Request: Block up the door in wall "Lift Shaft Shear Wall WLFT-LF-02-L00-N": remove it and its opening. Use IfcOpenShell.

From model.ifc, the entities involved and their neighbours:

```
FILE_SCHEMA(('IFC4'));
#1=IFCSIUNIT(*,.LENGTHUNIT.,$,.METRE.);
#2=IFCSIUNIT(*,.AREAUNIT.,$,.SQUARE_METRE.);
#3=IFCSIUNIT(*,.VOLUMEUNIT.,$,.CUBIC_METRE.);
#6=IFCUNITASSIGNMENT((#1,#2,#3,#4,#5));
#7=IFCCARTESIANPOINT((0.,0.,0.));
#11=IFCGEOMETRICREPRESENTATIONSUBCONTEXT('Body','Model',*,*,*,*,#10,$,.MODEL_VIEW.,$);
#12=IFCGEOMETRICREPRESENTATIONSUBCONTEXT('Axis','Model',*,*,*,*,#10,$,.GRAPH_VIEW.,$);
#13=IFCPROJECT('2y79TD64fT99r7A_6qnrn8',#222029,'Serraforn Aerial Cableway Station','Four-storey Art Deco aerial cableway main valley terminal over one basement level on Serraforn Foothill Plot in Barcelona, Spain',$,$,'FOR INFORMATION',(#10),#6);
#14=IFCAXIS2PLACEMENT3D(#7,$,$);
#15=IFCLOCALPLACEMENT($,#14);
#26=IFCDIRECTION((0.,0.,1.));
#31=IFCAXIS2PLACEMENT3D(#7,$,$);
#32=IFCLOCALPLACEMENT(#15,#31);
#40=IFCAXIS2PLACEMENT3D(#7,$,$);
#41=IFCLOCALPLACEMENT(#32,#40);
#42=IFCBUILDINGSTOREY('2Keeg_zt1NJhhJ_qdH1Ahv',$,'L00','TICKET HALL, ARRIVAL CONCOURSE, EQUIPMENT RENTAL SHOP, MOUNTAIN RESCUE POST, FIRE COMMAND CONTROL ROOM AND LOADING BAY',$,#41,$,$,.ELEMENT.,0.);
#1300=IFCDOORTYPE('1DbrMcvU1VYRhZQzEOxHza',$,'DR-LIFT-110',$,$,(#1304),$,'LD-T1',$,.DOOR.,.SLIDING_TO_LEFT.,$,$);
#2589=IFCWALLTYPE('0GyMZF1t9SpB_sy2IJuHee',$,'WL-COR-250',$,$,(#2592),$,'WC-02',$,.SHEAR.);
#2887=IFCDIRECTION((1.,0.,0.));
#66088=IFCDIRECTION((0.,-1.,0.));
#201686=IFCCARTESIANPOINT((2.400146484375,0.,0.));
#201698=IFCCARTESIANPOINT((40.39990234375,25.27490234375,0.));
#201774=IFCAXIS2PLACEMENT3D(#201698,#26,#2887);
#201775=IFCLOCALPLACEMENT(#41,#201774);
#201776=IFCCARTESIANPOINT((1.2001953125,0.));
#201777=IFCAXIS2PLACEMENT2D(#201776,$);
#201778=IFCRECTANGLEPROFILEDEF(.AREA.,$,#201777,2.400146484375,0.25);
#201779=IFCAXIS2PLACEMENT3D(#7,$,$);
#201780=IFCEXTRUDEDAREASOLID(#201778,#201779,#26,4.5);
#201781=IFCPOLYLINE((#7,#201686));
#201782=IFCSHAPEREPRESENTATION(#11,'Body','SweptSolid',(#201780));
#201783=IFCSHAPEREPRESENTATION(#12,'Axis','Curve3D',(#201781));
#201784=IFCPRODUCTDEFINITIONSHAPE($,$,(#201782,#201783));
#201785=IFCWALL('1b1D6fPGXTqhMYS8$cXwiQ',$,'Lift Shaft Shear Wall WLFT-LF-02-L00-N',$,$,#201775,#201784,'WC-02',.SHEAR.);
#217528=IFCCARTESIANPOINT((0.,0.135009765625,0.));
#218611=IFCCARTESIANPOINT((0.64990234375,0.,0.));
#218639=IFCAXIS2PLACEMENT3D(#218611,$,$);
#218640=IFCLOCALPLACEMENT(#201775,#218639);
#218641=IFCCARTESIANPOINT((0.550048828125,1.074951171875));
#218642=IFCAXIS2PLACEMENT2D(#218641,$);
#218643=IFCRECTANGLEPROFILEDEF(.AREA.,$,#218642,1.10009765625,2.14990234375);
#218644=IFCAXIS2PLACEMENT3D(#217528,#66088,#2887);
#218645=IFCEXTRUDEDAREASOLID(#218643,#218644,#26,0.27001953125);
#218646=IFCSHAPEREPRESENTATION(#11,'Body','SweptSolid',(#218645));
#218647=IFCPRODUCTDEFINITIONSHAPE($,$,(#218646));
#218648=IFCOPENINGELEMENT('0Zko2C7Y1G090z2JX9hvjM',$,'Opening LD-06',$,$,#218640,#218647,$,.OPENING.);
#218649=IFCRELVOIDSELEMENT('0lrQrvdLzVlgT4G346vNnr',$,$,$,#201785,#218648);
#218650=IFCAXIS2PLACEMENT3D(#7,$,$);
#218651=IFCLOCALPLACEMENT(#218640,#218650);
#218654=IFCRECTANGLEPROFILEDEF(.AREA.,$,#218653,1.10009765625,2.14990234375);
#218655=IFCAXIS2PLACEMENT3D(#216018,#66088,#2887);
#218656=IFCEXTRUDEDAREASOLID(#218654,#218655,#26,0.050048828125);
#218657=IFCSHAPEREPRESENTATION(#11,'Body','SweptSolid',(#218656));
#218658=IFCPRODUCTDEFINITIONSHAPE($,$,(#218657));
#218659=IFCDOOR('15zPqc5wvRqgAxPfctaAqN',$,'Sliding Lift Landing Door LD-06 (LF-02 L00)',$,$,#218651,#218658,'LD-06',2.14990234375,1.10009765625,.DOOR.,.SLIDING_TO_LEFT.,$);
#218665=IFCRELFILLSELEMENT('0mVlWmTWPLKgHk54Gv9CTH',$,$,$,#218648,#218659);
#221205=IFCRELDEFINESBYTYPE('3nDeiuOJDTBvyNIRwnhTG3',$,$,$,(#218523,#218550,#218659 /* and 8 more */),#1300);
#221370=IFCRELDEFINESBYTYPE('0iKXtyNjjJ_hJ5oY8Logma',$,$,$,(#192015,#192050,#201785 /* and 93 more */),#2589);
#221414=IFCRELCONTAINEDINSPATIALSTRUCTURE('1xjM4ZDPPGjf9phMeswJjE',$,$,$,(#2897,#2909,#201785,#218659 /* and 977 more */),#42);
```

```python
import ifcopenshell
import ifcopenshell.api.feature
import ifcopenshell.api.root
import ifcopenshell.geom
import ifcopenshell.util.shape

model = ifcopenshell.open("model.ifc")
settings = ifcopenshell.geom.settings()


def volume(element):
    """Net volume in cubic metres, openings subtracted."""
    shape = ifcopenshell.geom.create_shape(settings, element)
    return ifcopenshell.util.shape.get_volume(shape.geometry)


door = model.by_id(218659)
opening = door.FillsVoids[0].RelatingOpeningElement
wall = opening.VoidsElements[0].RelatingBuildingElement
before = volume(wall)

ifcopenshell.api.root.remove_product(model, product=door)
ifcopenshell.api.feature.remove_feature(model, feature=opening)

after = volume(wall)

print(f"wall volume {before:.3f} -> {after:.3f} m3")

model.write("model_updated.ifc")
```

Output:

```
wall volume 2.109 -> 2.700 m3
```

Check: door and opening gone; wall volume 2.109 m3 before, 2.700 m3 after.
